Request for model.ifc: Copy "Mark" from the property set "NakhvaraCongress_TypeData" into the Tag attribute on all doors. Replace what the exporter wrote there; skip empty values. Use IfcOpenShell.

First a look at what the model holds.

```python
import ifcopenshell
import ifcopenshell.util.element

model = ifcopenshell.open("model.ifc")
print(model.schema)
doors = model.by_type("IfcDoor")
print(len(doors), "doors")
for e in doors[:8]:
    source = ifcopenshell.util.element.get_pset(e, "NakhvaraCongress_TypeData", "Mark")
    target = e.Tag
    print(e.id(), repr(source), repr(target), sep=" | ")
```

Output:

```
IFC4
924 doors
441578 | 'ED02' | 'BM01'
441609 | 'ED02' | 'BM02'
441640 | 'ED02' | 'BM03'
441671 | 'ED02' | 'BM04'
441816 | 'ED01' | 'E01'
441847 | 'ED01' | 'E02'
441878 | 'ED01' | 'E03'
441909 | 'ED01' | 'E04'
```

```python
import ifcopenshell
import ifcopenshell.util.element

model = ifcopenshell.open("model.ifc")

count = 0
for e in model.by_type("IfcDoor"):
    value = ifcopenshell.util.element.get_pset(e, "NakhvaraCongress_TypeData", "Mark")
    current = e.Tag
    if not value or not value.strip() or current == value:
        continue
    e.Tag = value
    count += 1

print(count, "doors updated")

model.write("model_v2.ifc")
```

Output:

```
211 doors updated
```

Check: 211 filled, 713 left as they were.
